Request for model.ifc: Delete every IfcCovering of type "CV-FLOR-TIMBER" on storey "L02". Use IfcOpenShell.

First a look at what the model holds.

```python
import ifcopenshell
import ifcopenshell.util.element

model = ifcopenshell.open("model.ifc")
print(model.schema)
storey = next(s for s in model.by_type("IfcBuildingStorey") if s.Name == "L02")
coverings = [e for e in ifcopenshell.util.element.get_decomposition(storey) if e.is_a("IfcCovering")]
seen = {}
for e in coverings:
    element_type = ifcopenshell.util.element.get_type(e)
    name = element_type.Name if element_type not in (None, e) else None
    seen[name] = seen.get(name, 0) + 1
for name, count in sorted(seen.items(), key=str):
    print(count, "x", name)
```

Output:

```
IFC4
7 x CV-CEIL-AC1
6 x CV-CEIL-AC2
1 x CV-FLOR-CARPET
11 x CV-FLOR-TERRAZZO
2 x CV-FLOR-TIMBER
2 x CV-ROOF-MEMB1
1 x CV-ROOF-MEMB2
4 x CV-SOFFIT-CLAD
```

```python
import ifcopenshell
import ifcopenshell.api.root
import ifcopenshell.util.element

model = ifcopenshell.open("model.ifc")

storey = next(s for s in model.by_type("IfcBuildingStorey") if s.Name == "L02")
coverings = [e for e in ifcopenshell.util.element.get_decomposition(storey) if e.is_a("IfcCovering")]
targets = [e for e in coverings if (t := ifcopenshell.util.element.get_type(e)) not in (None, e) and t.Name == "CV-FLOR-TIMBER"]

for e in targets:
    ifcopenshell.api.root.remove_product(model, product=e)
print(len(targets), "removed")

model.write("model_rev.ifc")
```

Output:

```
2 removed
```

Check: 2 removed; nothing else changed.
